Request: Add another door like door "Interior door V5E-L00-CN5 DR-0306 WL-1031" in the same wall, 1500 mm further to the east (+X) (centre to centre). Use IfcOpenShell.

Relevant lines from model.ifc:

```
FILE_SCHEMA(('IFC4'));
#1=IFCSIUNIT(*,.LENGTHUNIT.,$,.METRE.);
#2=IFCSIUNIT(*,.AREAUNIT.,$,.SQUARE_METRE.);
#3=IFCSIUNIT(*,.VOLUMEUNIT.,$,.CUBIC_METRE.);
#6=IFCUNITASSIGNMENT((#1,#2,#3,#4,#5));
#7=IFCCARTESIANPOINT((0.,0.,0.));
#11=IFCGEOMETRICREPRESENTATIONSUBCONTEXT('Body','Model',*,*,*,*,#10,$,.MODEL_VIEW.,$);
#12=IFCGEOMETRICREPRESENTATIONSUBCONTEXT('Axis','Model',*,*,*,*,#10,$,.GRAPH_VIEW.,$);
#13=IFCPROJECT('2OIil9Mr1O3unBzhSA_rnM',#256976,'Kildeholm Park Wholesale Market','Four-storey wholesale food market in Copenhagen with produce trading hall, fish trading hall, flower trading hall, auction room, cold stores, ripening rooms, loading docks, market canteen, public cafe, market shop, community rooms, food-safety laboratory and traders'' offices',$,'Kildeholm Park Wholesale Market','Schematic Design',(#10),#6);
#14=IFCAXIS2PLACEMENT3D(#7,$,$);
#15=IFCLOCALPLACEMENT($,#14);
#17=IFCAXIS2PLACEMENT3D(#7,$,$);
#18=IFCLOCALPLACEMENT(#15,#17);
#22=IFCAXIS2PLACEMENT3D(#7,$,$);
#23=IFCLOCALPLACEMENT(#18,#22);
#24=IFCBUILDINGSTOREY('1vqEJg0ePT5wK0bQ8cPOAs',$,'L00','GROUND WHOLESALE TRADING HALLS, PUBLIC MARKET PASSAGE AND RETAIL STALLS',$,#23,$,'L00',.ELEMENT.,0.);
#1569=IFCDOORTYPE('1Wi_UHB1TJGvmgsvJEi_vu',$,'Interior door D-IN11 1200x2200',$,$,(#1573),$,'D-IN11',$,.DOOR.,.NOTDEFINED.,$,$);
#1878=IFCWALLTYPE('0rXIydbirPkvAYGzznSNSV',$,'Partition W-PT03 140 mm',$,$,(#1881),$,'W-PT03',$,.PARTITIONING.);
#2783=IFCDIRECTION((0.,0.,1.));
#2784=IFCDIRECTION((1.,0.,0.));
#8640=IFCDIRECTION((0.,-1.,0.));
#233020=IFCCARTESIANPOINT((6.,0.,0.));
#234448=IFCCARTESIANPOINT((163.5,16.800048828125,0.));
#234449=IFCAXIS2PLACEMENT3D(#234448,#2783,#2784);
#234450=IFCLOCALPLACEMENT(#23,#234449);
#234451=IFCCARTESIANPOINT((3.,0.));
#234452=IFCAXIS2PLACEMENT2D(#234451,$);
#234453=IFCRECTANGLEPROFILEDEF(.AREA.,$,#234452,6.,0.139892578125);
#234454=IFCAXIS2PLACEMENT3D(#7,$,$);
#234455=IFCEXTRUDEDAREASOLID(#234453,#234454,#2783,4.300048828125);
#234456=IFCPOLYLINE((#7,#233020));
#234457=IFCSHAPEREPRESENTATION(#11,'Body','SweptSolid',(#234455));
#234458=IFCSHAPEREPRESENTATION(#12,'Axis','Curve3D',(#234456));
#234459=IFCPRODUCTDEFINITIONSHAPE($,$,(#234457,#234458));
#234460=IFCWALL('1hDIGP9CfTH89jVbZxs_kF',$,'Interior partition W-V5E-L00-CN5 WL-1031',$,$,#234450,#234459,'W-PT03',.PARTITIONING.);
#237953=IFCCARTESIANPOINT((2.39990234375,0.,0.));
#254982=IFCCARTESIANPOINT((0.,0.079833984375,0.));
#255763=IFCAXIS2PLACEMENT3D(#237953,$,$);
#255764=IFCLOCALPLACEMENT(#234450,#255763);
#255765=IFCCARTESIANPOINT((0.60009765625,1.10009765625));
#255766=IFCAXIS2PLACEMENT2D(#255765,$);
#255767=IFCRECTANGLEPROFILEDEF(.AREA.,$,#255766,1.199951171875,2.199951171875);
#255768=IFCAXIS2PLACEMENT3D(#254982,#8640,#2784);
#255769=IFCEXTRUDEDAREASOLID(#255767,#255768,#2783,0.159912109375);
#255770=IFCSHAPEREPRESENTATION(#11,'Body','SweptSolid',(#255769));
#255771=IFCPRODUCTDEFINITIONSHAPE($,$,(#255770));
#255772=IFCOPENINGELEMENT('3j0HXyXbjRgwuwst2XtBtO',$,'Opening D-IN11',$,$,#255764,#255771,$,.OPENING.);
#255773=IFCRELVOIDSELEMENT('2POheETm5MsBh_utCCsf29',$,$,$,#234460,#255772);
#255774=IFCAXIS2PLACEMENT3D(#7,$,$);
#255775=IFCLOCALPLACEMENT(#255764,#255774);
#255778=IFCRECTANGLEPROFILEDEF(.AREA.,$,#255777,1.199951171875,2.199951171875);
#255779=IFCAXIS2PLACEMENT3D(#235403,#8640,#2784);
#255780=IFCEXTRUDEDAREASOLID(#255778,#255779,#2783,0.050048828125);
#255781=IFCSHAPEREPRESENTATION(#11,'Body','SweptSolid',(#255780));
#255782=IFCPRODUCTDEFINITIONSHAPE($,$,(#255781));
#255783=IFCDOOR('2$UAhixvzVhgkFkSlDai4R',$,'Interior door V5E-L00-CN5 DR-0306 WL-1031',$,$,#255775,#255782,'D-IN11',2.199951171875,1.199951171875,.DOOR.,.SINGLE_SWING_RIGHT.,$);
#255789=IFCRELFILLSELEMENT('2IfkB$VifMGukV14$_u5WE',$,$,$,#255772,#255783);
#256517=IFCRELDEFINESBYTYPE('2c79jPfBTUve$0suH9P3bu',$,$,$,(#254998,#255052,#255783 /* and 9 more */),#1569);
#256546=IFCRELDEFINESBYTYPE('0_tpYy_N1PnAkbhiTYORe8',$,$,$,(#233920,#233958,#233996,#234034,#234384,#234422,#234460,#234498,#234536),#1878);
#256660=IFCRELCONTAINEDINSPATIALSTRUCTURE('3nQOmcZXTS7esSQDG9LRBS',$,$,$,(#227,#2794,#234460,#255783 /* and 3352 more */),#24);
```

```python
import ifcopenshell
import ifcopenshell.api.feature
import ifcopenshell.api.geometry
import ifcopenshell.api.root
import ifcopenshell.geom
import ifcopenshell.util.element
import ifcopenshell.util.placement
import ifcopenshell.util.shape
import ifcopenshell.util.unit

model = ifcopenshell.open("model.ifc")
unit_scale = ifcopenshell.util.unit.calculate_unit_scale(model)
settings = ifcopenshell.geom.settings()


def volume(element):
    """Net volume in cubic metres, openings subtracted."""
    shape = ifcopenshell.geom.create_shape(settings, element)
    return ifcopenshell.util.shape.get_volume(shape.geometry)


door = model.by_guid("2$UAhixvzVhgkFkSlDai4R")
opening = door.FillsVoids[0].RelatingOpeningElement
wall = opening.VoidsElements[0].RelatingBuildingElement
before = volume(wall)
shift = ifcopenshell.util.placement.get_local_placement(wall.ObjectPlacement)[:3, 0] * 1.5 / unit_scale

# copy_class copies the void relationship, type, container and properties, but no geometry.
new_opening = ifcopenshell.api.root.copy_class(model, product=opening)
new_opening.Representation = ifcopenshell.util.element.copy_deep(
    model, opening.Representation, exclude=["IfcGeometricRepresentationContext", "IfcRepresentationMap"]
)
new_door = ifcopenshell.api.root.copy_class(model, product=door)
new_door.Representation = ifcopenshell.util.element.copy_deep(
    model, door.Representation, exclude=["IfcGeometricRepresentationContext", "IfcRepresentationMap"]
)
new_door.Tag = None
ifcopenshell.api.feature.add_filling(model, opening=new_opening, element=new_door)

for old, new in ((opening, new_opening), (door, new_door)):
    matrix = ifcopenshell.util.placement.get_local_placement(old.ObjectPlacement)
    matrix[:3, 3] += shift
    ifcopenshell.api.geometry.edit_object_placement(model, product=new, matrix=matrix, is_si=False)

after = volume(wall)

print(f"wall volume {before:.3f} -> {after:.3f} m3")

model.write("model_edited.ifc")
```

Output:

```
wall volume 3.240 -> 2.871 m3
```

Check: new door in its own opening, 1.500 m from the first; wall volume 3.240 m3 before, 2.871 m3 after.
